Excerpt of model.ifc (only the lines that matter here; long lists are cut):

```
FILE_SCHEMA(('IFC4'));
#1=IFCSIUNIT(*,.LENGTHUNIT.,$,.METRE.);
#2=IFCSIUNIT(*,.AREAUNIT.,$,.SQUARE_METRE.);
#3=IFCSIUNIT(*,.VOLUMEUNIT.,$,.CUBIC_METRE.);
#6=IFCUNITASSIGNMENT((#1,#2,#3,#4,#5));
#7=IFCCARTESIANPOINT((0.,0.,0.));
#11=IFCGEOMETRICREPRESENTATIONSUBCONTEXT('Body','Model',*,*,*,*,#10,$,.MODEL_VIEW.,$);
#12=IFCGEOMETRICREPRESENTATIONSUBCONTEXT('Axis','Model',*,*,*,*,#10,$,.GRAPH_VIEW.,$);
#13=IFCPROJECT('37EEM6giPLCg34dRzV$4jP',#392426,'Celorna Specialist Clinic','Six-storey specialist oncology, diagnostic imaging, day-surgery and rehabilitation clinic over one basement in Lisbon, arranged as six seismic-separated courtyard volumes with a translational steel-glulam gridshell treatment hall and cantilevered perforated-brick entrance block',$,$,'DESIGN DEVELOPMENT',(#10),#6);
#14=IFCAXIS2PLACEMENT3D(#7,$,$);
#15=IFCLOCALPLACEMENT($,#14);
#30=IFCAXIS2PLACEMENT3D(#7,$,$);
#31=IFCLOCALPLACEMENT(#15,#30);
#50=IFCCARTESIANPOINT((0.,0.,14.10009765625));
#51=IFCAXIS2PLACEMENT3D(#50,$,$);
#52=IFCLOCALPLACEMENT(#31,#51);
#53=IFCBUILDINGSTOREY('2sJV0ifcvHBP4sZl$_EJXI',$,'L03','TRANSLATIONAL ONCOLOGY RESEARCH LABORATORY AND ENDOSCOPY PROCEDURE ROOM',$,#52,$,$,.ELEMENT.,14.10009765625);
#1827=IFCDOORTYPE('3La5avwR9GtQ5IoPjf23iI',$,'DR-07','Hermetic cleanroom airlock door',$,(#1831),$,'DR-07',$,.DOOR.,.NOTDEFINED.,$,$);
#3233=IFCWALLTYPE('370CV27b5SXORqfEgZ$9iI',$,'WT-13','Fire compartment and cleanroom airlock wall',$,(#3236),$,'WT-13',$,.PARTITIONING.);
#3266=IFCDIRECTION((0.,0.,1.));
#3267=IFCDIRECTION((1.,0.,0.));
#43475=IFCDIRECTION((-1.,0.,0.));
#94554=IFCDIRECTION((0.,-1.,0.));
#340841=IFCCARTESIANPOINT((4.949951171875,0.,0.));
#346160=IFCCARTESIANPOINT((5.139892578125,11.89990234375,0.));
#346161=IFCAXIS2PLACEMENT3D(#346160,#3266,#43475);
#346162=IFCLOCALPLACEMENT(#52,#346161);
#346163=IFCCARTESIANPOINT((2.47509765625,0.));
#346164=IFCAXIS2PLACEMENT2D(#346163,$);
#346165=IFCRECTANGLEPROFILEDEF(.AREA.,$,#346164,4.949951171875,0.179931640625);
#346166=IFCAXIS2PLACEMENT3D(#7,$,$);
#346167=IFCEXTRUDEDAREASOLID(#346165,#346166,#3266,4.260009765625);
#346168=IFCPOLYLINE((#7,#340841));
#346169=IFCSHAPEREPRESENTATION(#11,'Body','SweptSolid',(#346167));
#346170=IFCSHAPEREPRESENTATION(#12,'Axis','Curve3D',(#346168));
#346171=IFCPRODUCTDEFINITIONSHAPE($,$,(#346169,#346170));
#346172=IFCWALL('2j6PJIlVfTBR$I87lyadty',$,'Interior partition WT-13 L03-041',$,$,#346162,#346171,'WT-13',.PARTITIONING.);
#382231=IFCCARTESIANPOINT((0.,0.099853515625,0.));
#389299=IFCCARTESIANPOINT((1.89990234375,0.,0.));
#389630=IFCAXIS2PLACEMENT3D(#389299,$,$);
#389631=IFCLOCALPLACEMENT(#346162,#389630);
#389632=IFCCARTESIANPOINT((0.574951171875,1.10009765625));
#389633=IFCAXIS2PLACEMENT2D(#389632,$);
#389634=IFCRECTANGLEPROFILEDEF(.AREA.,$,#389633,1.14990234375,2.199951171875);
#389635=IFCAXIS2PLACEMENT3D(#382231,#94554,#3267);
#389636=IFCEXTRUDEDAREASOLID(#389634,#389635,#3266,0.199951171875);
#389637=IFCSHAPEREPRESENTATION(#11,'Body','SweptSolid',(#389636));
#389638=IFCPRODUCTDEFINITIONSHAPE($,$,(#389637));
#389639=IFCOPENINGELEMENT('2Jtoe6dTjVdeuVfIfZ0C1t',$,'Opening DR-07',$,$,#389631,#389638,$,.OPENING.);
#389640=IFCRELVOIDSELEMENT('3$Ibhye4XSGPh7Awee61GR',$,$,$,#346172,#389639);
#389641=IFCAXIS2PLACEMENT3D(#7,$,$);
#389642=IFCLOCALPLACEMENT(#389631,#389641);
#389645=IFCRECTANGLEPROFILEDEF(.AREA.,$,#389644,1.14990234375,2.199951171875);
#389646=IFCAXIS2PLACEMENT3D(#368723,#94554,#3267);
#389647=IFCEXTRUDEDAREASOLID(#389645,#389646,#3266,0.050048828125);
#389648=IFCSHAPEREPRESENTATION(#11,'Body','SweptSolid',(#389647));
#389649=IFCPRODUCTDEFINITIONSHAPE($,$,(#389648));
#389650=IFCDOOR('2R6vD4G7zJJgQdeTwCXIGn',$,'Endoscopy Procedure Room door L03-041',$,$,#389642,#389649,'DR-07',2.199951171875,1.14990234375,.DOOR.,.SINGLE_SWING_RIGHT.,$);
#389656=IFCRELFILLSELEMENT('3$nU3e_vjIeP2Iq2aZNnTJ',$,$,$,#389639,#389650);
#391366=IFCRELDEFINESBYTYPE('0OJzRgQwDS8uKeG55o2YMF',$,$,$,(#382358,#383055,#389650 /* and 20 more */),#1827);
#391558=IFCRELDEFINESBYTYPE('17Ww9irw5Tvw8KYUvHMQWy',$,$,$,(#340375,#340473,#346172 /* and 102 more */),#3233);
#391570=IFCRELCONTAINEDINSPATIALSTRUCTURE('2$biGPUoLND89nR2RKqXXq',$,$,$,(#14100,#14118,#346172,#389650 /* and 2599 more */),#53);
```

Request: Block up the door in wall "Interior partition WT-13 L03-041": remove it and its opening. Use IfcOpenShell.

```python
import ifcopenshell
import ifcopenshell.api.feature
import ifcopenshell.api.root
import ifcopenshell.geom
import ifcopenshell.util.shape

model = ifcopenshell.open("model.ifc")
settings = ifcopenshell.geom.settings()


def volume(element):
    """Net volume in cubic metres, openings subtracted."""
    shape = ifcopenshell.geom.create_shape(settings, element)
    return ifcopenshell.util.shape.get_volume(shape.geometry)


door = model.by_guid("2R6vD4G7zJJgQdeTwCXIGn")
opening = door.FillsVoids[0].RelatingOpeningElement
wall = opening.VoidsElements[0].RelatingBuildingElement
before = volume(wall)

ifcopenshell.api.root.remove_product(model, product=door)
ifcopenshell.api.feature.remove_feature(model, feature=opening)

after = volume(wall)

print(f"wall volume {before:.3f} -> {after:.3f} m3")

model.write("model_v2.ifc")
```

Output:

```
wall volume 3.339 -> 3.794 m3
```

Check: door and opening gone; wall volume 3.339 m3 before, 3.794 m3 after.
